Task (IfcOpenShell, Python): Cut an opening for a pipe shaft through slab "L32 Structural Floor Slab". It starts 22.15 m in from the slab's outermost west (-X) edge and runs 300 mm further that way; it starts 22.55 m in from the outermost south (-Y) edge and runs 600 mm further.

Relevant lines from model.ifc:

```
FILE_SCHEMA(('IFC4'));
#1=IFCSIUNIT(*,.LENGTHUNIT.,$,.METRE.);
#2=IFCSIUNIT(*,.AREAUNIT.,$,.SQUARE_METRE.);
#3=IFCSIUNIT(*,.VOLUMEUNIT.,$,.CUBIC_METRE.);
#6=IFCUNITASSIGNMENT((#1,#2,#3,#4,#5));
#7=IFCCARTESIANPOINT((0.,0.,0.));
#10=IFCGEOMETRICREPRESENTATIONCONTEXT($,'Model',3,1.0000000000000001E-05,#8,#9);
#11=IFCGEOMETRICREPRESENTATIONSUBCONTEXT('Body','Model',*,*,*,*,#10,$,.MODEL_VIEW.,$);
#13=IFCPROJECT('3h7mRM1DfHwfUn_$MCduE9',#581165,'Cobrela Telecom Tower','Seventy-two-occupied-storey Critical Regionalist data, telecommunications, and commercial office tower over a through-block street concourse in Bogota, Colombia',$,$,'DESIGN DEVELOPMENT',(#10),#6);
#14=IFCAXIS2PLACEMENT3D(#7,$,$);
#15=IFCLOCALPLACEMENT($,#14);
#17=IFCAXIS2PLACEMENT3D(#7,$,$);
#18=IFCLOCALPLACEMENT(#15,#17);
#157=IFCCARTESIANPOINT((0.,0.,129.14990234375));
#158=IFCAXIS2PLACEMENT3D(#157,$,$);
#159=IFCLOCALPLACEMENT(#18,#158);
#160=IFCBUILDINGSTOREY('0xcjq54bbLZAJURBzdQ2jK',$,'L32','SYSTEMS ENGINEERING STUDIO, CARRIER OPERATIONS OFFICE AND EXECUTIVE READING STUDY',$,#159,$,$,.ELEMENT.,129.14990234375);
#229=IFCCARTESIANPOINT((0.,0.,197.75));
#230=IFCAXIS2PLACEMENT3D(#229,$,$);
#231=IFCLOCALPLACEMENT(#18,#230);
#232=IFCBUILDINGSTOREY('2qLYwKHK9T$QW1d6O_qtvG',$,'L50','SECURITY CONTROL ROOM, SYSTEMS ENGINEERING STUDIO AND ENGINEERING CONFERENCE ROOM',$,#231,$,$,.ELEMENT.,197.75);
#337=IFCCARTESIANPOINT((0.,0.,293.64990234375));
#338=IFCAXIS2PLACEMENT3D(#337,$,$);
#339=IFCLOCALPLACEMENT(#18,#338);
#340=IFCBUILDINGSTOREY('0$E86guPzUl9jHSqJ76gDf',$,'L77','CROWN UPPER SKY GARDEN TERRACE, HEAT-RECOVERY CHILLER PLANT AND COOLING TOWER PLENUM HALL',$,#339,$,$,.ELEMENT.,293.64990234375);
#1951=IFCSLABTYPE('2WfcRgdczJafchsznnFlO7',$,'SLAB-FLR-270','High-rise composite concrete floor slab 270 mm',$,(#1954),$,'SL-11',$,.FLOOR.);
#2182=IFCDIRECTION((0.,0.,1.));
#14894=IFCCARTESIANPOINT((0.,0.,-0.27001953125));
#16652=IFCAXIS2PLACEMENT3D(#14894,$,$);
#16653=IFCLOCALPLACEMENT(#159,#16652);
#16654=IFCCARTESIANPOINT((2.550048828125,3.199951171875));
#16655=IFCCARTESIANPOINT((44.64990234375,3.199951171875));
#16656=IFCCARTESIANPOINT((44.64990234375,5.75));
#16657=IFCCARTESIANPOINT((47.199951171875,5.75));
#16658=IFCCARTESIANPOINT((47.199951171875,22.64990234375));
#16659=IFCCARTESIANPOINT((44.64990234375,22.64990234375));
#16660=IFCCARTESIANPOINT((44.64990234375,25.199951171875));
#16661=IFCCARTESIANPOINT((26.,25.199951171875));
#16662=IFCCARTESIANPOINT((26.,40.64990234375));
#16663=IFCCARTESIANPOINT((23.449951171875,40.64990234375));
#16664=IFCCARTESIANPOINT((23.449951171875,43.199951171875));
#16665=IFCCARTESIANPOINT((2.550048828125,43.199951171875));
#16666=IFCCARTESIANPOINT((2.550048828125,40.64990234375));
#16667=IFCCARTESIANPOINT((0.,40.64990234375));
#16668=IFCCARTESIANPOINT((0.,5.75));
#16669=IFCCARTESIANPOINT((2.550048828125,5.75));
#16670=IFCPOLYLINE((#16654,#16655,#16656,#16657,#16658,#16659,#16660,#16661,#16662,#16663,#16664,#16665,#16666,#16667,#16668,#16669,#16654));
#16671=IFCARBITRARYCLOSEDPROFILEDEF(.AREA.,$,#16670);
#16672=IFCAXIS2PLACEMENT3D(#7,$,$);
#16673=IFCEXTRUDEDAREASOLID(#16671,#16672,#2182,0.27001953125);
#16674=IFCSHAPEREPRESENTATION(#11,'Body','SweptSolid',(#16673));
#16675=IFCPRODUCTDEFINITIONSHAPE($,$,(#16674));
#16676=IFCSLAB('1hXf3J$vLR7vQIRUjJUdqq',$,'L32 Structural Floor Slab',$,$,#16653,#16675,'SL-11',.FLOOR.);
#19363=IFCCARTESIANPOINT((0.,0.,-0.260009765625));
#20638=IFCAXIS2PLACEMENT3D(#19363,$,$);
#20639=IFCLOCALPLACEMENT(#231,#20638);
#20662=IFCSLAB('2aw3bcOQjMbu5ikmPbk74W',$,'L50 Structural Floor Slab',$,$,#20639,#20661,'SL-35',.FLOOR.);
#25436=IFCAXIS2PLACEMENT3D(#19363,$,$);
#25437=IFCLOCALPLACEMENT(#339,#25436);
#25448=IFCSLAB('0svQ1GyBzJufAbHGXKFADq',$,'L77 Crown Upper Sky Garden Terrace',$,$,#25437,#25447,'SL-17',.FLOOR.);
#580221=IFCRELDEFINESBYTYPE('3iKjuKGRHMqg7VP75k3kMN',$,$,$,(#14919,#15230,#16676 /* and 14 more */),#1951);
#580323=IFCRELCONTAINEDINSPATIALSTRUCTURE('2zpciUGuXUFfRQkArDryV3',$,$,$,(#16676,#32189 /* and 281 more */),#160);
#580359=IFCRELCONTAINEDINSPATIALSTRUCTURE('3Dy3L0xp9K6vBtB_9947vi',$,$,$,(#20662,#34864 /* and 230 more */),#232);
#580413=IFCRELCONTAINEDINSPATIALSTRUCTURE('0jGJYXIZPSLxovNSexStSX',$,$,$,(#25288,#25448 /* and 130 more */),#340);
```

```python
import numpy as np
import ifcopenshell
import ifcopenshell.api.feature
import ifcopenshell.api.geometry
import ifcopenshell.api.root
import ifcopenshell.geom
import ifcopenshell.util.placement
import ifcopenshell.util.representation
import ifcopenshell.util.shape
import ifcopenshell.util.unit

model = ifcopenshell.open("model.ifc")
unit_scale = ifcopenshell.util.unit.calculate_unit_scale(model)
settings = ifcopenshell.geom.settings()


def volume(element):
    """Net volume in cubic metres, openings subtracted."""
    shape = ifcopenshell.geom.create_shape(settings, element)
    return ifcopenshell.util.shape.get_volume(shape.geometry)


slab = model.by_guid("1hXf3J$vLR7vQIRUjJUdqq")
before = volume(slab)

# Extent in the slab's own axes, in metres. The edges named are its -X and -Y sides.
slab_shape = ifcopenshell.geom.create_shape(settings, slab)
vertices = ifcopenshell.util.shape.get_vertices(slab_shape.geometry)
x_min, y_min, bottom = vertices.min(axis=0)
top = vertices[:, 2].max()

opening = ifcopenshell.api.root.create_entity(model, ifc_class="IfcOpeningElement", name="Pipe shaft opening", predefined_type="OPENING")
context = ifcopenshell.util.representation.get_context(model, "Model", "Body", "MODEL_VIEW")
width, depth = 0.3, 0.6
outline = [(0.0, 0.0), (width, 0.0), (width, depth), (0.0, depth), (0.0, 0.0)]
# Overshoot both faces by 50 mm so the cut is clean.
shape = ifcopenshell.api.geometry.add_slab_representation(
    model, context=context, depth=top - bottom + 0.1, polyline=outline
)
ifcopenshell.api.geometry.assign_representation(model, product=opening, representation=shape)

matrix = ifcopenshell.util.placement.get_local_placement(slab.ObjectPlacement)
matrix[:, 3] = matrix @ np.append(np.array([x_min + 22.15, y_min + 22.55, bottom - 0.05]) / unit_scale, 1.0)
ifcopenshell.api.geometry.edit_object_placement(model, product=opening, matrix=matrix, is_si=False)
ifcopenshell.api.feature.add_feature(model, feature=opening, element=slab)

after = volume(slab)

print(f"slab volume {before:.3f} -> {after:.3f} m3")

model.write("model_updated.ifc")
```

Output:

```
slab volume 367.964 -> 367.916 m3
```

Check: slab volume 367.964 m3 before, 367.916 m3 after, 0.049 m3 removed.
